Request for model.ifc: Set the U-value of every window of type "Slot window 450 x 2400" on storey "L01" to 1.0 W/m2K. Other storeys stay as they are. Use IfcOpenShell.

First a look at what the model holds.

```python
import ifcopenshell
import ifcopenshell.util.element

model = ifcopenshell.open("model.ifc")
print(model.schema)
storey = next(s for s in model.by_type("IfcBuildingStorey") if s.Name == "L01")
windows = [e for e in ifcopenshell.util.element.get_decomposition(storey) if e.is_a("IfcWindow")]
seen = {}
for e in windows:
    element_type = ifcopenshell.util.element.get_type(e)
    key = (element_type.Name if element_type != e and element_type else None, ifcopenshell.util.element.get_pset(e, "Pset_WindowCommon", "ThermalTransmittance"))
    seen[key] = seen.get(key, 0) + 1
for (name, value), count in sorted(seen.items(), key=str):
    print(count, "x", name, "|", value)
```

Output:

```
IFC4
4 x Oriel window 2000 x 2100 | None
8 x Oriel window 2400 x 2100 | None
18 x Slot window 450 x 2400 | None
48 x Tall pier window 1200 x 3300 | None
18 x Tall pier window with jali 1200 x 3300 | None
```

```python
import ifcopenshell
import ifcopenshell.api.pset
import ifcopenshell.util.element

model = ifcopenshell.open("model.ifc")

storey = next(s for s in model.by_type("IfcBuildingStorey") if s.Name == "L01")
windows = [e for e in ifcopenshell.util.element.get_decomposition(storey) if e.is_a("IfcWindow")]

count = 0
for e in windows:
    element_type = ifcopenshell.util.element.get_type(e)
    if element_type in (None, e) or element_type.Name != "Slot window 450 x 2400":
        continue
    # add_pset returns the element's existing set when there is one.
    pset = ifcopenshell.api.pset.add_pset(model, product=e, name="Pset_WindowCommon")
    ifcopenshell.api.pset.edit_pset(model, pset=pset, properties={"ThermalTransmittance": 1.0})
    count += 1

print(count, "windows updated")

model.write("model_v2.ifc")
```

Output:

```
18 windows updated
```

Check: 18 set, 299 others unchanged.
